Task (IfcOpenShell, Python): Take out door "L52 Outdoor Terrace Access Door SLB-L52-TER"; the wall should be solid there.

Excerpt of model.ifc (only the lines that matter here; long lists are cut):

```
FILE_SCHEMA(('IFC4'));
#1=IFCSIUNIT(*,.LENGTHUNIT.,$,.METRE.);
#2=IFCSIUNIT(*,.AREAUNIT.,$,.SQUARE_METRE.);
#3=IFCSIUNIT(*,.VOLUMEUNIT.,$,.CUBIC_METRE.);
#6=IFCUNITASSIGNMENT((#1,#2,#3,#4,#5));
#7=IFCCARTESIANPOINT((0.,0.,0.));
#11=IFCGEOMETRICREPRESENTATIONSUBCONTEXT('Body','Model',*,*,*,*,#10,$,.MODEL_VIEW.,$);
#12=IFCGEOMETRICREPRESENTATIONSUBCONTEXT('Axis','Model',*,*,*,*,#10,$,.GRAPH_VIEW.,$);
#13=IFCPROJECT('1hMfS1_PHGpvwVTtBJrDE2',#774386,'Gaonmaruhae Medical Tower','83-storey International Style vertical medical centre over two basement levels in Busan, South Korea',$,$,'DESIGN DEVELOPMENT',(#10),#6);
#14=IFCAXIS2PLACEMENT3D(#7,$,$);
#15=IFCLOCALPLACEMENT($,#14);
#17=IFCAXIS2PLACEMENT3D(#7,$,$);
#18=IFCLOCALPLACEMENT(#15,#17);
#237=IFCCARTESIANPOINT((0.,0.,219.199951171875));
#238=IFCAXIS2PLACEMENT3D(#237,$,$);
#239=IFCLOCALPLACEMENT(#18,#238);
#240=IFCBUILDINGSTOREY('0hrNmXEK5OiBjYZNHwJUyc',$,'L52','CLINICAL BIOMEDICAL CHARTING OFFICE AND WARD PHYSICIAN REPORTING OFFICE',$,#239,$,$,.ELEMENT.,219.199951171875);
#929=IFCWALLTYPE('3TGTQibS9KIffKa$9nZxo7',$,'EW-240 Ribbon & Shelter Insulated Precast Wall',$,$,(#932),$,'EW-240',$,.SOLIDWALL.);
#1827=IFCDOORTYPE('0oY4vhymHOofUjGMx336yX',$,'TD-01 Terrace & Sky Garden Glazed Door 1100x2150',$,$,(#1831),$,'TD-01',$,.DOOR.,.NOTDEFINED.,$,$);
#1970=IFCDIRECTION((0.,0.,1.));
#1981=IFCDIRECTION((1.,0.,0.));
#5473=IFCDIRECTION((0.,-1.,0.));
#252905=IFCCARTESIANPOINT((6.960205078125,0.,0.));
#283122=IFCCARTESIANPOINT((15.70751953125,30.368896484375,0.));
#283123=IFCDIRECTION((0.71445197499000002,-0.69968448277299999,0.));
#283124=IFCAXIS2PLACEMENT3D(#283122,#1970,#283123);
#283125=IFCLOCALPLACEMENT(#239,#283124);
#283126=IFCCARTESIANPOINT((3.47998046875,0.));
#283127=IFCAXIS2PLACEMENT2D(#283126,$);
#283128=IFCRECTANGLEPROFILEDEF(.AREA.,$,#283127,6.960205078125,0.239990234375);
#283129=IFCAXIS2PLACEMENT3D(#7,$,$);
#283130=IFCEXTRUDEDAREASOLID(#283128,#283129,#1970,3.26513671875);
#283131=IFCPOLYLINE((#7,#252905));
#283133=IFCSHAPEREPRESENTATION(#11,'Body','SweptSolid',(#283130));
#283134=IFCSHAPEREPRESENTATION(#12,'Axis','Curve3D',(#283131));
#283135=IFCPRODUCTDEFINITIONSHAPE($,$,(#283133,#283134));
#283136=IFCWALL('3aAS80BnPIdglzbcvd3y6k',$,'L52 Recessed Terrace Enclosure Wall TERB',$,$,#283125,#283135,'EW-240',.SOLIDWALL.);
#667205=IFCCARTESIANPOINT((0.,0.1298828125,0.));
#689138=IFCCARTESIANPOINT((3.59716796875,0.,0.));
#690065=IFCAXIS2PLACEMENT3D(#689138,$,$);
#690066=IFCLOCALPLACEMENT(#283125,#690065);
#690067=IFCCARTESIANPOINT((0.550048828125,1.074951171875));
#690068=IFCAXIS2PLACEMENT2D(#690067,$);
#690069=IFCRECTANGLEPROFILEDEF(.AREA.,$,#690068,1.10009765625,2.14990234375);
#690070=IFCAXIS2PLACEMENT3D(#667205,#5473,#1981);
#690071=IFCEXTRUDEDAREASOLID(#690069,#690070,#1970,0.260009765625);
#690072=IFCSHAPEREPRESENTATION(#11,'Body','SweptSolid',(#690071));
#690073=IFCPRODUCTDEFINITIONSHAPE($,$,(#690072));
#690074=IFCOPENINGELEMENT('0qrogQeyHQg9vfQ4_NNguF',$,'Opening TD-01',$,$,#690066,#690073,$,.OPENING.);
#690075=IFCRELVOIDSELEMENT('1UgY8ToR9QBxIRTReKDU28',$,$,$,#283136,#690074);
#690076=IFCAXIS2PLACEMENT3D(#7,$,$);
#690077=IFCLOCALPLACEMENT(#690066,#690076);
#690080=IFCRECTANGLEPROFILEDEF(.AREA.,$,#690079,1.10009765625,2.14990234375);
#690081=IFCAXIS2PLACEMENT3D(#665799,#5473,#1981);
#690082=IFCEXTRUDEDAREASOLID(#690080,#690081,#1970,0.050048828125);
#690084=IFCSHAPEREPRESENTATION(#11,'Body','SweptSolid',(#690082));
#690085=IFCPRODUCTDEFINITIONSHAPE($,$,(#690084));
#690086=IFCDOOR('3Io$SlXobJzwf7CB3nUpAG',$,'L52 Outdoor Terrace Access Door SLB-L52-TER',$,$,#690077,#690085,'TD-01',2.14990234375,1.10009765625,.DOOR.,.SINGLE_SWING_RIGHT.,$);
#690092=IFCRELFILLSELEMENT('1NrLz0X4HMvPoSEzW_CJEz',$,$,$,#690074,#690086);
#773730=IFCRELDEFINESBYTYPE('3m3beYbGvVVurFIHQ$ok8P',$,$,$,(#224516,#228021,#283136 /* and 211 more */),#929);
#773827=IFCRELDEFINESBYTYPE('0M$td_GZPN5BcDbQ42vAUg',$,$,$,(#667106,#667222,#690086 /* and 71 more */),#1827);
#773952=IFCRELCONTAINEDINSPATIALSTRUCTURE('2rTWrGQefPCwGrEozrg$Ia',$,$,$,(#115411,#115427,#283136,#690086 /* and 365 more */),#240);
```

```python
import ifcopenshell
import ifcopenshell.api.feature
import ifcopenshell.api.root
import ifcopenshell.geom
import ifcopenshell.util.shape

model = ifcopenshell.open("model.ifc")
settings = ifcopenshell.geom.settings()


def volume(element):
    """Net volume in cubic metres, openings subtracted."""
    shape = ifcopenshell.geom.create_shape(settings, element)
    return ifcopenshell.util.shape.get_volume(shape.geometry)


door = model.by_guid("3Io$SlXobJzwf7CB3nUpAG")
opening = door.FillsVoids[0].RelatingOpeningElement
wall = opening.VoidsElements[0].RelatingBuildingElement
before = volume(wall)

ifcopenshell.api.root.remove_product(model, product=door)
ifcopenshell.api.feature.remove_feature(model, feature=opening)

after = volume(wall)

print(f"wall volume {before:.3f} -> {after:.3f} m3")

model.write("model_edited.ifc")
```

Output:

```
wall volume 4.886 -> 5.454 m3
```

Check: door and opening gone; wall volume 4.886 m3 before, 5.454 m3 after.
